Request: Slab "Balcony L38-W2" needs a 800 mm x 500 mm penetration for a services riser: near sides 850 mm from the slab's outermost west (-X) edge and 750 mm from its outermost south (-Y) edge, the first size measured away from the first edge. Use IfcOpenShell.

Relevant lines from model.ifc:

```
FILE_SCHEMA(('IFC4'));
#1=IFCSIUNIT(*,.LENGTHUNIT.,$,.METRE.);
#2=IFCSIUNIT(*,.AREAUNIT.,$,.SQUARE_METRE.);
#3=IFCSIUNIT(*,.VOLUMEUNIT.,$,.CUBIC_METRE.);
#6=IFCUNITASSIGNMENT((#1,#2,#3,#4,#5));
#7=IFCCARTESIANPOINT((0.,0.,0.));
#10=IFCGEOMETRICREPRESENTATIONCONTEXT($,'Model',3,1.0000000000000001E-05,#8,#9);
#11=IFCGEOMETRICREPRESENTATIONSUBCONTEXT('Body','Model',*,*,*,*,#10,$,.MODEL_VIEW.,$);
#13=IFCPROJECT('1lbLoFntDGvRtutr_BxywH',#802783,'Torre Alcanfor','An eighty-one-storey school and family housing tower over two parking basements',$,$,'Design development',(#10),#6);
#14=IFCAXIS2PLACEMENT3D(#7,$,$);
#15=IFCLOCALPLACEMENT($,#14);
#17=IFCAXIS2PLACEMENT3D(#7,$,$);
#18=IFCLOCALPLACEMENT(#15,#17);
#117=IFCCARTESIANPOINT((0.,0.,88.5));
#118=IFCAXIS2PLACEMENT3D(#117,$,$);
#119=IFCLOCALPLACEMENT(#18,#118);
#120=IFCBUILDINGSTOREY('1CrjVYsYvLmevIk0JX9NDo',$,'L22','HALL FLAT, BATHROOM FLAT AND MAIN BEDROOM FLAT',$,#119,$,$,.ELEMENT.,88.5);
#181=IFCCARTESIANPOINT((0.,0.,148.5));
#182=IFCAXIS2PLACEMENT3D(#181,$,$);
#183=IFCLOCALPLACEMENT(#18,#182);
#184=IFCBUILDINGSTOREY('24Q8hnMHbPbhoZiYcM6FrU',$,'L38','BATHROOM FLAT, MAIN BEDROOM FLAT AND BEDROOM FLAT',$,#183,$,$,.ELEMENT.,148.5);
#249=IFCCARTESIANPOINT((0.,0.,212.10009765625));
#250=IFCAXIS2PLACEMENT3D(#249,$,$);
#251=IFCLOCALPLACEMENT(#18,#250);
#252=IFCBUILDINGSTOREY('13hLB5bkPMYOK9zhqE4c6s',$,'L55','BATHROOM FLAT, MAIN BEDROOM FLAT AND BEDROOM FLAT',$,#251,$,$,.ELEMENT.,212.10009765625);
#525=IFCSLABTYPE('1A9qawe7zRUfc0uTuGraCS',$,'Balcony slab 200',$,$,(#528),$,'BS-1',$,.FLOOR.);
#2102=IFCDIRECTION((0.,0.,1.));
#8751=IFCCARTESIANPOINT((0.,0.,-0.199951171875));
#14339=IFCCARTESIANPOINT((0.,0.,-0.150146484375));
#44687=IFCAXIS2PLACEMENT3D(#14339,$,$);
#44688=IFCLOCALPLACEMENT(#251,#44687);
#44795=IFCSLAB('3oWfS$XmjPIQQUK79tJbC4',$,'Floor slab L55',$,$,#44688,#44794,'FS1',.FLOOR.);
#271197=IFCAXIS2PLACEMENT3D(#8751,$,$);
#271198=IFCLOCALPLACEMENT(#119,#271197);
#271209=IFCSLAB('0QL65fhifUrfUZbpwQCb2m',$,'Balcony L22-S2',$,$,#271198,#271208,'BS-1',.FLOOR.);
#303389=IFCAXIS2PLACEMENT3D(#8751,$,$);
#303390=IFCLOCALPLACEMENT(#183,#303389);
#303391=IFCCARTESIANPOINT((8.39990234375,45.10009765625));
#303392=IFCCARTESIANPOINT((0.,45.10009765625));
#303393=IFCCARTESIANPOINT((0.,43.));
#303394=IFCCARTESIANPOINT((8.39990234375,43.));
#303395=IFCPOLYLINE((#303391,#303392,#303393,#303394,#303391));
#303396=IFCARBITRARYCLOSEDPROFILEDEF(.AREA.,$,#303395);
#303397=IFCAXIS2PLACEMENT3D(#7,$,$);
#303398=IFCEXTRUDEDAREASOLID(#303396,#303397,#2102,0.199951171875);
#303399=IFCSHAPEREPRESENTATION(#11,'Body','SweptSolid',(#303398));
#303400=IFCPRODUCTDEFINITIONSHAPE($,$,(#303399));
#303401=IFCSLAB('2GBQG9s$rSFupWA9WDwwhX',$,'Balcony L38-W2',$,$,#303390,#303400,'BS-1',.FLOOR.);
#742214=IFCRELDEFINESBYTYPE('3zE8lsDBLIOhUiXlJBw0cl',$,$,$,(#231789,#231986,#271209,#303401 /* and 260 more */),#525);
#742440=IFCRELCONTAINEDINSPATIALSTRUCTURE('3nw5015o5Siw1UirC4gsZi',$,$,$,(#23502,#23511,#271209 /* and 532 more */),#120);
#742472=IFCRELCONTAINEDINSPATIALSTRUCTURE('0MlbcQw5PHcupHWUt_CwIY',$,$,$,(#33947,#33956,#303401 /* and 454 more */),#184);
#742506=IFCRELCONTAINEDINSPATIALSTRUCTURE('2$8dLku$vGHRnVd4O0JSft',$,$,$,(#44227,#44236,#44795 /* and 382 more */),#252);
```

```python
import numpy as np
import ifcopenshell
import ifcopenshell.api.feature
import ifcopenshell.api.geometry
import ifcopenshell.api.root
import ifcopenshell.geom
import ifcopenshell.util.placement
import ifcopenshell.util.representation
import ifcopenshell.util.shape
import ifcopenshell.util.unit

model = ifcopenshell.open("model.ifc")
unit_scale = ifcopenshell.util.unit.calculate_unit_scale(model)
settings = ifcopenshell.geom.settings()


def volume(element):
    """Net volume in cubic metres, openings subtracted."""
    shape = ifcopenshell.geom.create_shape(settings, element)
    return ifcopenshell.util.shape.get_volume(shape.geometry)


slab = model.by_guid("2GBQG9s$rSFupWA9WDwwhX")
before = volume(slab)

# Extent in the slab's own axes, in metres. The edges named are its -X and -Y sides.
slab_shape = ifcopenshell.geom.create_shape(settings, slab)
vertices = ifcopenshell.util.shape.get_vertices(slab_shape.geometry)
x_min, y_min, bottom = vertices.min(axis=0)
top = vertices[:, 2].max()

opening = ifcopenshell.api.root.create_entity(model, ifc_class="IfcOpeningElement", name="Services riser opening", predefined_type="OPENING")
context = ifcopenshell.util.representation.get_context(model, "Model", "Body", "MODEL_VIEW")
width, depth = 0.8, 0.5
outline = [(0.0, 0.0), (width, 0.0), (width, depth), (0.0, depth), (0.0, 0.0)]
# Overshoot both faces by 50 mm so the cut is clean.
shape = ifcopenshell.api.geometry.add_slab_representation(
    model, context=context, depth=top - bottom + 0.1, polyline=outline
)
ifcopenshell.api.geometry.assign_representation(model, product=opening, representation=shape)

matrix = ifcopenshell.util.placement.get_local_placement(slab.ObjectPlacement)
matrix[:, 3] = matrix @ np.append(np.array([x_min + 0.85, y_min + 0.75, bottom - 0.05]) / unit_scale, 1.0)
ifcopenshell.api.geometry.edit_object_placement(model, product=opening, matrix=matrix, is_si=False)
ifcopenshell.api.feature.add_feature(model, feature=opening, element=slab)

after = volume(slab)

print(f"slab volume {before:.3f} -> {after:.3f} m3")

model.write("model-out.ifc")
```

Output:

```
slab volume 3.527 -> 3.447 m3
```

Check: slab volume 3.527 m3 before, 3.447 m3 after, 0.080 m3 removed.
